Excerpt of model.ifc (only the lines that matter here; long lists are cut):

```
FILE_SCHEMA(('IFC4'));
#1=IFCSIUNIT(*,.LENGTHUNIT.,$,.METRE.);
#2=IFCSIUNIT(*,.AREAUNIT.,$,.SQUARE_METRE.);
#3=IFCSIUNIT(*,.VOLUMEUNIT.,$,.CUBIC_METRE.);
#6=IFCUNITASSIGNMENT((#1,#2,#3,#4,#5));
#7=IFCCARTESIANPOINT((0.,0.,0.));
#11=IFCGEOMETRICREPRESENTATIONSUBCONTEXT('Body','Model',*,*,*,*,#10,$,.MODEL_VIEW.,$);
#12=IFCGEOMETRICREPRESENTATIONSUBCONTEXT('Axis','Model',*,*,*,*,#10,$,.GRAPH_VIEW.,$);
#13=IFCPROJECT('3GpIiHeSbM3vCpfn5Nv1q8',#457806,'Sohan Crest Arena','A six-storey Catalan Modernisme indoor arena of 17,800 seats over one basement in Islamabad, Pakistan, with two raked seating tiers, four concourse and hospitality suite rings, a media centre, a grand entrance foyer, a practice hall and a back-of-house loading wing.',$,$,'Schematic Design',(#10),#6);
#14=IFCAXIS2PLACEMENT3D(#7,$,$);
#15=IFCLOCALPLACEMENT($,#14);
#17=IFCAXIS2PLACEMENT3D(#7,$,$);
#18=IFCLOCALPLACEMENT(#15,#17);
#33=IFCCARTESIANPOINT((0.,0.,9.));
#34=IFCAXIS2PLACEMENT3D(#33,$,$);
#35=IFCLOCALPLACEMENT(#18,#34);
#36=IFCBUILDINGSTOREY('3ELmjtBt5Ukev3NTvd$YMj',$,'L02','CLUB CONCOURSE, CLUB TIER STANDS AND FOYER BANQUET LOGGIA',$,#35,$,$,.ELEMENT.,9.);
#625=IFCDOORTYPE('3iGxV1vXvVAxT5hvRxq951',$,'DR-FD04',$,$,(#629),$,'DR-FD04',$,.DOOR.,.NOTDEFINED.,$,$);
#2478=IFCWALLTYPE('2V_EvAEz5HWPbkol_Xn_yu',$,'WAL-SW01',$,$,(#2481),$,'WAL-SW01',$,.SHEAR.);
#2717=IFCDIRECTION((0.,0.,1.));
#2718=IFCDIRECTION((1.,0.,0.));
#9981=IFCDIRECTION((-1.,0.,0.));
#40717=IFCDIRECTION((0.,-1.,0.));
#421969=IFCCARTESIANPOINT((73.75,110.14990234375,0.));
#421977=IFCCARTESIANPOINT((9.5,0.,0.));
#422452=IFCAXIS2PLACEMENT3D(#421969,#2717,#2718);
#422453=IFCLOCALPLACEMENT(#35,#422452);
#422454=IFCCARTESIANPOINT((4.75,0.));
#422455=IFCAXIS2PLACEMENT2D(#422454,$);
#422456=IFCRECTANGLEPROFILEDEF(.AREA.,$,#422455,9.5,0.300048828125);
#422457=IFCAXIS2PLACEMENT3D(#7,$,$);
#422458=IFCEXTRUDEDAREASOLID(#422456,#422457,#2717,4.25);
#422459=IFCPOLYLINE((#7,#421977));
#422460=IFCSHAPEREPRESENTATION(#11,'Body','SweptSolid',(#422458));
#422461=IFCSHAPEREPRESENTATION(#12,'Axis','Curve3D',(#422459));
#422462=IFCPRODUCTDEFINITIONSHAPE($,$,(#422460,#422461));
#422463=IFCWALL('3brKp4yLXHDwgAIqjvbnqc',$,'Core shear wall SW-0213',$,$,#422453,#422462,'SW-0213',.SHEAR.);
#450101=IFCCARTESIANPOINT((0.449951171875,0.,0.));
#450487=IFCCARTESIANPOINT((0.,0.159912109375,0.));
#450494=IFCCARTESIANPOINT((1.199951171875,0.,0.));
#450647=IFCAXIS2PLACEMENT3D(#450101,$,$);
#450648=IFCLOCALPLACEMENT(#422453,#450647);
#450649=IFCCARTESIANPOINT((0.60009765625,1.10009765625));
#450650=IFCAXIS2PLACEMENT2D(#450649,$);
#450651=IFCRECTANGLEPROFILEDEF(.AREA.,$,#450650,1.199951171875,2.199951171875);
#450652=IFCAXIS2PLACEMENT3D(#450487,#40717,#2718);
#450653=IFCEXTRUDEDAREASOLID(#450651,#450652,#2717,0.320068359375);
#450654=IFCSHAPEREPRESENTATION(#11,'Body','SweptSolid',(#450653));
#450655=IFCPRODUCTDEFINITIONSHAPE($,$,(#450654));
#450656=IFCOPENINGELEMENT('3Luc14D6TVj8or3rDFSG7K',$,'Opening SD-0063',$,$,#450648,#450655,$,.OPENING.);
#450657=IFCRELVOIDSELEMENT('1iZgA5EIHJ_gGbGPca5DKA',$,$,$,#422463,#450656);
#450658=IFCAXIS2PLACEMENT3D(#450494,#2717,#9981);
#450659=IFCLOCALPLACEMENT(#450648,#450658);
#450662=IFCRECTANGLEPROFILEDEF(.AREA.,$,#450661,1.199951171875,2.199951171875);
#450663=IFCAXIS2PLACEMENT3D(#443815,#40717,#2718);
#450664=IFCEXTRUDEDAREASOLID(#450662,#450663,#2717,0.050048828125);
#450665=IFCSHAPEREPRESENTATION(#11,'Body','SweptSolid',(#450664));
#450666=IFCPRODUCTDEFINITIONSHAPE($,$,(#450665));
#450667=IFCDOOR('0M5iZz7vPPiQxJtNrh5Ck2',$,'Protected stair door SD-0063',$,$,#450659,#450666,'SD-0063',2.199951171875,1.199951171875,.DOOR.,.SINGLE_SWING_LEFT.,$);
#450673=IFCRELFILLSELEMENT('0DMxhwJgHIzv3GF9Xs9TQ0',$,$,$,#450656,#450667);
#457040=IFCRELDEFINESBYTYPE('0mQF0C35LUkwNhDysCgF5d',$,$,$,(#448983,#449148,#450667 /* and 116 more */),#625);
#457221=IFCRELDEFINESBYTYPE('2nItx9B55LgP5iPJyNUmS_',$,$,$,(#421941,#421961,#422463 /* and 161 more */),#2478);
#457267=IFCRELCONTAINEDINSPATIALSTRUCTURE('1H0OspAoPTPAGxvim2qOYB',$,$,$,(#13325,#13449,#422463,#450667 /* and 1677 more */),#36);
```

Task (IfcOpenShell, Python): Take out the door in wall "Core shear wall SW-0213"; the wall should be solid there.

```python
import ifcopenshell
import ifcopenshell.api.feature
import ifcopenshell.api.root
import ifcopenshell.geom
import ifcopenshell.util.shape

model = ifcopenshell.open("model.ifc")
settings = ifcopenshell.geom.settings()


def volume(element):
    """Net volume in cubic metres, openings subtracted."""
    shape = ifcopenshell.geom.create_shape(settings, element)
    return ifcopenshell.util.shape.get_volume(shape.geometry)


door = model.by_guid("0M5iZz7vPPiQxJtNrh5Ck2")
opening = door.FillsVoids[0].RelatingOpeningElement
wall = opening.VoidsElements[0].RelatingBuildingElement
before = volume(wall)

ifcopenshell.api.root.remove_product(model, product=door)
ifcopenshell.api.feature.remove_feature(model, feature=opening)

after = volume(wall)

print(f"wall volume {before:.3f} -> {after:.3f} m3")

model.write("model_rev.ifc")
```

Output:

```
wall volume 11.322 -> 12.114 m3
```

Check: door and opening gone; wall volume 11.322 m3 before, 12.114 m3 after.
